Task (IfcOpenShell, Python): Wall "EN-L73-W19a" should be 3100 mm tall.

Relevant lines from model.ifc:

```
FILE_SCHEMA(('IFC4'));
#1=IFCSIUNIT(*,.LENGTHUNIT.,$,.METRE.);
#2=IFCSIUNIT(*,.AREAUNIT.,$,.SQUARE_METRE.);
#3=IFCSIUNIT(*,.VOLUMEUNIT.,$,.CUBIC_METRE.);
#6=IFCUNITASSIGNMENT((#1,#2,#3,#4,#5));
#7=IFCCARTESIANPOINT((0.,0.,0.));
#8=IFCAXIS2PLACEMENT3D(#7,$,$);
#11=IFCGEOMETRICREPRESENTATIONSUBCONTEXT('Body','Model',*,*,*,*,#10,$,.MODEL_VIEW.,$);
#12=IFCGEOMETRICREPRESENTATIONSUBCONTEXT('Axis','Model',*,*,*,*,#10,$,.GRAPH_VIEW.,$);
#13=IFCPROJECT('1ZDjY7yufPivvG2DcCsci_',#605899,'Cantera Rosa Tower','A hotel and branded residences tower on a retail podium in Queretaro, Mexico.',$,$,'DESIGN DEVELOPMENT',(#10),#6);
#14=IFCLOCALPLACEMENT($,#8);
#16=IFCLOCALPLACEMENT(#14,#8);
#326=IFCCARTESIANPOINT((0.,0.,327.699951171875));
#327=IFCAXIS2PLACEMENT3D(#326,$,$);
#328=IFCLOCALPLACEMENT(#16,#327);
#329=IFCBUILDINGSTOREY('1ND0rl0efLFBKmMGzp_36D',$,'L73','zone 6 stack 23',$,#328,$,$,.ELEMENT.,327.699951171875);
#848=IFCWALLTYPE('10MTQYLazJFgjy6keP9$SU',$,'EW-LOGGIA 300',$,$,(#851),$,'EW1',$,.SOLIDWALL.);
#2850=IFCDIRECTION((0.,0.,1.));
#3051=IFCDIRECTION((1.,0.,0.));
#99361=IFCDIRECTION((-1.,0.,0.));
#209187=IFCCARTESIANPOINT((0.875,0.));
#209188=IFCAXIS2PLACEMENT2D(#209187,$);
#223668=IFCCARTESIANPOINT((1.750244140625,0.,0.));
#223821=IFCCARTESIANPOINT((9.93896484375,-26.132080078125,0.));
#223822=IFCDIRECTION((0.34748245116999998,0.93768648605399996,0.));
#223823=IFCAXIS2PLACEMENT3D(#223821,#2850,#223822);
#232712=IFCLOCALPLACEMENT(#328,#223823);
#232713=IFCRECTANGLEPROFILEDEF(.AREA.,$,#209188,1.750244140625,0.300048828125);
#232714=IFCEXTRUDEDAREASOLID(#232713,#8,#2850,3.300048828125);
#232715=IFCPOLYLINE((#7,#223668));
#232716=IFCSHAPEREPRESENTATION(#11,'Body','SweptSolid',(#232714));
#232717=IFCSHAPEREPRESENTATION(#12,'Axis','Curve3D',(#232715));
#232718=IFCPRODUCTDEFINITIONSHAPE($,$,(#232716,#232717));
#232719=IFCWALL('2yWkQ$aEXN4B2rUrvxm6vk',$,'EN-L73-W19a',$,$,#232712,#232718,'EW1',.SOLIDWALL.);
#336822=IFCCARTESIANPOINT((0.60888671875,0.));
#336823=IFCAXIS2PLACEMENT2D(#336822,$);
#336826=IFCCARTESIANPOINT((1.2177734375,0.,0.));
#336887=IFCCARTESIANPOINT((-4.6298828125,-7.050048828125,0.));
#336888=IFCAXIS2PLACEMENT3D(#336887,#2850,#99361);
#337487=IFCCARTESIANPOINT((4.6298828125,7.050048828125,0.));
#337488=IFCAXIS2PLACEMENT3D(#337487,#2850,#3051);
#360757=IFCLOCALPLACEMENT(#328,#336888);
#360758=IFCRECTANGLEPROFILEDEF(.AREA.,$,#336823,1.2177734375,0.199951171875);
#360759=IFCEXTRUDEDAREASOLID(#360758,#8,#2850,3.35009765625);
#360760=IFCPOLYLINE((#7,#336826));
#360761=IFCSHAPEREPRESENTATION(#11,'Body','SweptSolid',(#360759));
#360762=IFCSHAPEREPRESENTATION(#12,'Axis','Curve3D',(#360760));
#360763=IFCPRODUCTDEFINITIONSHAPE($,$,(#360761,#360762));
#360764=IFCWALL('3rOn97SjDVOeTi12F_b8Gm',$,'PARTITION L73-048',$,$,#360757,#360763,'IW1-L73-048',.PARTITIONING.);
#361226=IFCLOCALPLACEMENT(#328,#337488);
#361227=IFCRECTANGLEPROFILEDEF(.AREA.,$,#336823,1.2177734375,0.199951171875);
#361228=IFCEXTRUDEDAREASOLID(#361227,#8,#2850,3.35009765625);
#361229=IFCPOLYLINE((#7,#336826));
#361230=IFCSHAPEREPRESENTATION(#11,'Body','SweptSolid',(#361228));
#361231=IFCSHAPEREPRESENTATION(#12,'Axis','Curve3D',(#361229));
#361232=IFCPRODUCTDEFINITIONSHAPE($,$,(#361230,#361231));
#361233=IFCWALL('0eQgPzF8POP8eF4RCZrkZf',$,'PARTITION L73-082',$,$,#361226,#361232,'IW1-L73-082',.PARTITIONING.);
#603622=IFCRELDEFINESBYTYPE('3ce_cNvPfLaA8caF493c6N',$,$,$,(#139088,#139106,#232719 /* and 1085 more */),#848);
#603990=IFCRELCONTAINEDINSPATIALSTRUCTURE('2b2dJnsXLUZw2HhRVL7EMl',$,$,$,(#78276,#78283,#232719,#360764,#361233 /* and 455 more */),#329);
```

```python
import ifcopenshell
import ifcopenshell.geom
import ifcopenshell.util.representation
import ifcopenshell.util.shape

model = ifcopenshell.open("model.ifc")
settings = ifcopenshell.geom.settings()


def volume(element):
    """Net volume in cubic metres, openings subtracted."""
    shape = ifcopenshell.geom.create_shape(settings, element)
    return ifcopenshell.util.shape.get_volume(shape.geometry)


wall = model.by_guid("2yWkQ$aEXN4B2rUrvxm6vk")
before = volume(wall)

body = ifcopenshell.util.representation.get_representation(wall, "Model", "Body")
solid = body.Items[0]
old_height = solid.Depth
solid.Depth = 3.1
after = volume(wall)

print(f"height {old_height:g} -> {solid.Depth:g}, volume {before:.3f} -> {after:.3f} m3")

model.write("model_v2.ifc")
```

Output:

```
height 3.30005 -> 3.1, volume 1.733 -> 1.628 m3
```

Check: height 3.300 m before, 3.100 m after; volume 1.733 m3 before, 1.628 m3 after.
